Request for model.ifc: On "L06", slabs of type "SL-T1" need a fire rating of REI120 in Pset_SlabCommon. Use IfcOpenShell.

First a look at what the model holds.

```python
import ifcopenshell
import ifcopenshell.util.element

model = ifcopenshell.open("model.ifc")
print(model.schema)
storey = next(s for s in model.by_type("IfcBuildingStorey") if s.Name == "L06")
slabs = [e for e in ifcopenshell.util.element.get_decomposition(storey) if e.is_a("IfcSlab")]
seen = {}
for e in slabs:
    element_type = ifcopenshell.util.element.get_type(e)
    key = (element_type.Name if element_type != e and element_type else None, ifcopenshell.util.element.get_pset(e, "Pset_SlabCommon", "FireRating"))
    seen[key] = seen.get(key, 0) + 1
for (name, value), count in sorted(seen.items(), key=str):
    print(count, "x", name, "|", value)
```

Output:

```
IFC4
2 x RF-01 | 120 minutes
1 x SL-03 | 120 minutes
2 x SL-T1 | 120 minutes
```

```python
import ifcopenshell
import ifcopenshell.api.pset
import ifcopenshell.util.element

model = ifcopenshell.open("model.ifc")

storey = next(s for s in model.by_type("IfcBuildingStorey") if s.Name == "L06")
slabs = [e for e in ifcopenshell.util.element.get_decomposition(storey) if e.is_a("IfcSlab")]

count = 0
for e in slabs:
    element_type = ifcopenshell.util.element.get_type(e)
    if element_type in (None, e) or element_type.Name != "SL-T1":
        continue
    # add_pset returns the element's existing set when there is one.
    pset = ifcopenshell.api.pset.add_pset(model, product=e, name="Pset_SlabCommon")
    ifcopenshell.api.pset.edit_pset(model, pset=pset, properties={"FireRating": "REI120"})
    count += 1

print(count, "slabs updated")

model.write("model-out.ifc")
```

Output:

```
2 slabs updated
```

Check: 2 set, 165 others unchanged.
